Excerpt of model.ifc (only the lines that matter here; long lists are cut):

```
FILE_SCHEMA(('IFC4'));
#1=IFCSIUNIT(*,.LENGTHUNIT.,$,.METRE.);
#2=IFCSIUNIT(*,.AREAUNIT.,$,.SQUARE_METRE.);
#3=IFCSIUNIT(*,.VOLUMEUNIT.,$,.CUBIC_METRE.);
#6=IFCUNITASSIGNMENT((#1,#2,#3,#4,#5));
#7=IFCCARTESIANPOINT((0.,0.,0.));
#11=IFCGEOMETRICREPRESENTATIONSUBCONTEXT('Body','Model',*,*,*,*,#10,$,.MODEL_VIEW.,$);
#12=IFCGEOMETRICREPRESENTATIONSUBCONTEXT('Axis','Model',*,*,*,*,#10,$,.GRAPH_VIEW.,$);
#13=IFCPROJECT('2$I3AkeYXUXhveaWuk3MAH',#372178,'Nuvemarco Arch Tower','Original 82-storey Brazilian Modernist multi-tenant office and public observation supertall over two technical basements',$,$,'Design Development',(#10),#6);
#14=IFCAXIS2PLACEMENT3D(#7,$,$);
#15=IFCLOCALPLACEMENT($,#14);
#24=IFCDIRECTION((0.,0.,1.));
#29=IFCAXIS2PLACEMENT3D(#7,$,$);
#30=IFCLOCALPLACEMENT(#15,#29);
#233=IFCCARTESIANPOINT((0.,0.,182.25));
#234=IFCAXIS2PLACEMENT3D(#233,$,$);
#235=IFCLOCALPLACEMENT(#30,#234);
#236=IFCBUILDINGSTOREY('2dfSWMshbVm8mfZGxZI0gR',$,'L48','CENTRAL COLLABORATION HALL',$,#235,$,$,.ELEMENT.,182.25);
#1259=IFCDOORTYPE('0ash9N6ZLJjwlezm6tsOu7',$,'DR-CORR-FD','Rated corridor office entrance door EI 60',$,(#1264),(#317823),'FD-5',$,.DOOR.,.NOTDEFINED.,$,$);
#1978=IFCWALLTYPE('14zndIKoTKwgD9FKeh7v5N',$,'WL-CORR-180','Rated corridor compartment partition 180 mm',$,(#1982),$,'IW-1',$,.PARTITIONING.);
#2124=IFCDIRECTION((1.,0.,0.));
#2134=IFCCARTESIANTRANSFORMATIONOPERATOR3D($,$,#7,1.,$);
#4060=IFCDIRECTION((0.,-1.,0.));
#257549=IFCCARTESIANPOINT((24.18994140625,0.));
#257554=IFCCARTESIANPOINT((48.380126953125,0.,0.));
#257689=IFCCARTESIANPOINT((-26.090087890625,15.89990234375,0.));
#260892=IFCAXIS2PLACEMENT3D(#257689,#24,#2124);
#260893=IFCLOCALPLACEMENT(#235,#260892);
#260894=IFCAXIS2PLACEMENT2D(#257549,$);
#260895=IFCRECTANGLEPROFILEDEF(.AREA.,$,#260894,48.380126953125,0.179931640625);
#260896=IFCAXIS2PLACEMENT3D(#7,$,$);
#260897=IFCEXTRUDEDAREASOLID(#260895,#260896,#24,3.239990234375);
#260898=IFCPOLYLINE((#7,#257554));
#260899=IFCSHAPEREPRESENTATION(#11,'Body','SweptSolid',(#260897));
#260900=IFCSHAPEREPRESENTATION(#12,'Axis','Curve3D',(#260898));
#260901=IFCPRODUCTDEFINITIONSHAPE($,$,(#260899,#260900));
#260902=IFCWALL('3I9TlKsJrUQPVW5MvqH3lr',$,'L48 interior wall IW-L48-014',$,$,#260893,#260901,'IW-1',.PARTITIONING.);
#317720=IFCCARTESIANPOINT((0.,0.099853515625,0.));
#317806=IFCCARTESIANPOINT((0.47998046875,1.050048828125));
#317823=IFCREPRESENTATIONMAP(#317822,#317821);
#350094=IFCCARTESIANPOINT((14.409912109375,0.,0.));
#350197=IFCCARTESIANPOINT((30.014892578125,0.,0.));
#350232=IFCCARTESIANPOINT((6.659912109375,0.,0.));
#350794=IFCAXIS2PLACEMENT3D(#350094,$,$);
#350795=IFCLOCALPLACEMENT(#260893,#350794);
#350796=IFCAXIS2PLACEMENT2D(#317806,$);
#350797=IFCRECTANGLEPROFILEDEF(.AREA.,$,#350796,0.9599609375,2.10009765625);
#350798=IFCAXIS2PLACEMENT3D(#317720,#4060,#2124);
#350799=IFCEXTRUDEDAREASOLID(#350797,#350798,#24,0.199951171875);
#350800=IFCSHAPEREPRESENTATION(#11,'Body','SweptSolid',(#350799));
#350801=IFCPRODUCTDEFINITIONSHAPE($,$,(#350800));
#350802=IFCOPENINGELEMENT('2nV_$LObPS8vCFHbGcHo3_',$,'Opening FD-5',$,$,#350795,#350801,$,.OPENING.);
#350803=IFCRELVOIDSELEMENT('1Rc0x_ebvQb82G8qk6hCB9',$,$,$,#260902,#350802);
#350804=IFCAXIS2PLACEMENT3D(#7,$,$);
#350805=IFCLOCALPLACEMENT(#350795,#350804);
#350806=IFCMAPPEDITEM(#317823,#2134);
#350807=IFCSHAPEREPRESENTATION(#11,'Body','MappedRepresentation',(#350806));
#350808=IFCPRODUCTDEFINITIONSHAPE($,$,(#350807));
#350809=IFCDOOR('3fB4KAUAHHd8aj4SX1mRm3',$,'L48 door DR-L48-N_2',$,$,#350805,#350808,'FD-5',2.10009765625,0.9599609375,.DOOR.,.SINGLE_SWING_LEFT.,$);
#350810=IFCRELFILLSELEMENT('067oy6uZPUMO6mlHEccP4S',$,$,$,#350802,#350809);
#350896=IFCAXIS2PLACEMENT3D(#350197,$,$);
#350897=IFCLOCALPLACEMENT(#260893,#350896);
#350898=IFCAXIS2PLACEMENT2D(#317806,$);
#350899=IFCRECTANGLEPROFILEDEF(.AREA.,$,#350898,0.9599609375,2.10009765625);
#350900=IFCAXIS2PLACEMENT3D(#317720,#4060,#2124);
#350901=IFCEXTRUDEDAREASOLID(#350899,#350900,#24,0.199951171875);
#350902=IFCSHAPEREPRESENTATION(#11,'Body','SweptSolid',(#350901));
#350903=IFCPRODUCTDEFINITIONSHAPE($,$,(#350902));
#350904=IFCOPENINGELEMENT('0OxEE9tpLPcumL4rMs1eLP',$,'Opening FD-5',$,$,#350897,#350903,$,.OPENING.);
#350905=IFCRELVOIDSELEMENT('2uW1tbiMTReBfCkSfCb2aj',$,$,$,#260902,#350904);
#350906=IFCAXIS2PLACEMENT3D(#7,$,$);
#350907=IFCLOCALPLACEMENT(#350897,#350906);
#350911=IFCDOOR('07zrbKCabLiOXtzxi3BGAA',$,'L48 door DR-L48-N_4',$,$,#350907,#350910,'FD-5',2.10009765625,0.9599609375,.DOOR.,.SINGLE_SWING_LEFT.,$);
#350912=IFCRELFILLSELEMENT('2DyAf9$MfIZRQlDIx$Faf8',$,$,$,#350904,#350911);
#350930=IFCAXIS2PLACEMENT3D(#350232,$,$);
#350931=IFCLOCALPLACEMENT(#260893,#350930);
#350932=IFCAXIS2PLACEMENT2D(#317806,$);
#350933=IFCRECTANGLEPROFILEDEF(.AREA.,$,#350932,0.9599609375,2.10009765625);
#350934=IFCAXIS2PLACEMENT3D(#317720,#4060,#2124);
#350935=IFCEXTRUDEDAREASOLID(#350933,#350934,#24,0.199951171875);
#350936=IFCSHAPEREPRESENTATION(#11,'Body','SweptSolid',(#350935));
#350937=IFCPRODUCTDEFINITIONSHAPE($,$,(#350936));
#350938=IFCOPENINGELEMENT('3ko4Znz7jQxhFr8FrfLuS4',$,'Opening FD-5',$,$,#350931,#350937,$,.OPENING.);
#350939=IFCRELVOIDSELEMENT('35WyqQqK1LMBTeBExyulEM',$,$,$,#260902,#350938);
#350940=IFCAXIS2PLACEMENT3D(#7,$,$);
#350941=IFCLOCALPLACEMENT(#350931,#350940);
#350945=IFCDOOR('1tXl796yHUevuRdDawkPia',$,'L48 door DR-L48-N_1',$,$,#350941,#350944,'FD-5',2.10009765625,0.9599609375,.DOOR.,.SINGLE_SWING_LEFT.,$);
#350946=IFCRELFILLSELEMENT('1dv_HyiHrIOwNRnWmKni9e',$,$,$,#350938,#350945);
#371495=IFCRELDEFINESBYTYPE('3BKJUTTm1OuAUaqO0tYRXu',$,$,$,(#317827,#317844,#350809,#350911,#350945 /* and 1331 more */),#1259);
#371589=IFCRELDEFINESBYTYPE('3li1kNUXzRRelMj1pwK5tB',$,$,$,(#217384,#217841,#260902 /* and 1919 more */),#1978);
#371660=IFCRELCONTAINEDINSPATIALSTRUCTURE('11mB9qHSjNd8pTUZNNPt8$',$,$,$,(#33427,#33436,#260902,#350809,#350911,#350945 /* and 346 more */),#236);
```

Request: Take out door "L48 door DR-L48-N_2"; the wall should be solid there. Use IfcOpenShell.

```python
import ifcopenshell
import ifcopenshell.api.feature
import ifcopenshell.api.root
import ifcopenshell.geom
import ifcopenshell.util.shape

model = ifcopenshell.open("model.ifc")
settings = ifcopenshell.geom.settings()


def volume(element):
    """Net volume in cubic metres, openings subtracted."""
    shape = ifcopenshell.geom.create_shape(settings, element)
    return ifcopenshell.util.shape.get_volume(shape.geometry)


door = model.by_guid("3fB4KAUAHHd8aj4SX1mRm3")
opening = door.FillsVoids[0].RelatingOpeningElement
wall = opening.VoidsElements[0].RelatingBuildingElement
before = volume(wall)

ifcopenshell.api.root.remove_product(model, product=door)
ifcopenshell.api.feature.remove_feature(model, feature=opening)

after = volume(wall)

print(f"wall volume {before:.3f} -> {after:.3f} m3")

model.write("model_v2.ifc")
```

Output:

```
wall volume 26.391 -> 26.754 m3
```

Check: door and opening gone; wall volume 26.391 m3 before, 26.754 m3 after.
